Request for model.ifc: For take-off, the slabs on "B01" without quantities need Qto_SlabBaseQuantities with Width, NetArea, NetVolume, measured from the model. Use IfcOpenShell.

First a look at what the model holds.

```python
import ifcopenshell
import ifcopenshell.util.element
import ifcopenshell.util.unit

model = ifcopenshell.open("model.ifc")
print(model.schema)
for unit_type in ("LENGTHUNIT", "AREAUNIT", "VOLUMEUNIT"):
    print(unit_type, ifcopenshell.util.unit.calculate_unit_scale(model, unit_type))
storey = next(s for s in model.by_type("IfcBuildingStorey") if s.Name == "B01")
slabs = [e for e in ifcopenshell.util.element.get_decomposition(storey) if e.is_a("IfcSlab")]
for e in sorted(slabs, key=lambda e: e.id()):
    print(e.id(), e.is_a(), e.Name, list(ifcopenshell.util.element.get_psets(e, qtos_only=True)), sep=" | ")
```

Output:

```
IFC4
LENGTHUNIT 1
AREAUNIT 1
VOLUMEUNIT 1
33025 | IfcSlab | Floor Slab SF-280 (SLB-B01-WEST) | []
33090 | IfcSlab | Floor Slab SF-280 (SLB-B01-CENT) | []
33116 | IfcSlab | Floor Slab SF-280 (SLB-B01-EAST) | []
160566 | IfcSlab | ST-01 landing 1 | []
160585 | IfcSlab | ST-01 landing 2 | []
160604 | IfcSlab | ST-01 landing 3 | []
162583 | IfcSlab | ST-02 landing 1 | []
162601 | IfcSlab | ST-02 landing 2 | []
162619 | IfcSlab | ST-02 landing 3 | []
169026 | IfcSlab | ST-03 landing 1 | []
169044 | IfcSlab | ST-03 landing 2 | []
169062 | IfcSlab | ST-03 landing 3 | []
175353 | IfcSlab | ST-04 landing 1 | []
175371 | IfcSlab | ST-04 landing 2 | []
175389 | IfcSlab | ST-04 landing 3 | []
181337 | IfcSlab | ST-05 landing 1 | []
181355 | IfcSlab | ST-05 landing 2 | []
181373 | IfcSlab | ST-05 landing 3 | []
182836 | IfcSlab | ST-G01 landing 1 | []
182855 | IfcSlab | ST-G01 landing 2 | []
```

```python
import ifcopenshell
import ifcopenshell.api.pset
import ifcopenshell.geom
import ifcopenshell.util.element
import ifcopenshell.util.shape
import ifcopenshell.util.unit

model = ifcopenshell.open("model.ifc")
unit_scale = ifcopenshell.util.unit.calculate_unit_scale(model)
area_scale = ifcopenshell.util.unit.calculate_unit_scale(model, "AREAUNIT")
volume_scale = ifcopenshell.util.unit.calculate_unit_scale(model, "VOLUMEUNIT")
settings = ifcopenshell.geom.settings()

storey = next(s for s in model.by_type("IfcBuildingStorey") if s.Name == "B01")
slabs = [e for e in ifcopenshell.util.element.get_decomposition(storey) if e.is_a("IfcSlab")]

for e in sorted(slabs, key=lambda e: e.id()):
    if ifcopenshell.util.element.get_psets(e, qtos_only=True, should_inherit=False):
        continue
    # Geometry comes back in metres, in the element's own axes.
    shape = ifcopenshell.geom.create_shape(settings, e)
    values = {
        "Width": ifcopenshell.util.shape.get_z(shape.geometry) / unit_scale,
        "NetArea": ifcopenshell.util.shape.get_footprint_area(shape.geometry) / area_scale,
        "NetVolume": ifcopenshell.util.shape.get_volume(shape.geometry) / volume_scale,
    }
    qto = ifcopenshell.api.pset.add_qto(model, product=e, name="Qto_SlabBaseQuantities")
    ifcopenshell.api.pset.edit_qto(model, qto=qto, properties=values)
    print(e.id(), {k: round(v, 3) for k, v in values.items()})

model.write("model_v2.ifc")
```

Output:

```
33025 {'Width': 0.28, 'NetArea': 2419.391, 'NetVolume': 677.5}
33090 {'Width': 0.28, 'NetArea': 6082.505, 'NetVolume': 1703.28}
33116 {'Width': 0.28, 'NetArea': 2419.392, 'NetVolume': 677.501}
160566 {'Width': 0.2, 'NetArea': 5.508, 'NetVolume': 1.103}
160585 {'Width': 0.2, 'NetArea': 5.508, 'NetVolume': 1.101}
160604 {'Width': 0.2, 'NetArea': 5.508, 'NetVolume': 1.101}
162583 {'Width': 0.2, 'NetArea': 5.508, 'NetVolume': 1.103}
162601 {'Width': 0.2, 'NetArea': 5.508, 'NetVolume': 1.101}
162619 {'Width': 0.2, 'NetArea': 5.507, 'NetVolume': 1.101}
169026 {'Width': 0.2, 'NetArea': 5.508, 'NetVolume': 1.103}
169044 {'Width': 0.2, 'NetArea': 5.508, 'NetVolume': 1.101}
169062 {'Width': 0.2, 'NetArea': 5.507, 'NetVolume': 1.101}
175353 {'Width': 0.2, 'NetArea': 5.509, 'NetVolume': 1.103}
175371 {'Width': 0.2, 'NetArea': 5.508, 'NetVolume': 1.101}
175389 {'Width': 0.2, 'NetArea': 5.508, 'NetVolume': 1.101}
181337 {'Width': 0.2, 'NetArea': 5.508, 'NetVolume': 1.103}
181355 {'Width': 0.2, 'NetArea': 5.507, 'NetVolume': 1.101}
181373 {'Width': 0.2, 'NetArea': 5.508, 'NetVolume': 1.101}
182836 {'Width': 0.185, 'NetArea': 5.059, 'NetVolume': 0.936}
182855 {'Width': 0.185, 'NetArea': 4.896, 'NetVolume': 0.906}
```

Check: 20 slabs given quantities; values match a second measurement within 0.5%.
